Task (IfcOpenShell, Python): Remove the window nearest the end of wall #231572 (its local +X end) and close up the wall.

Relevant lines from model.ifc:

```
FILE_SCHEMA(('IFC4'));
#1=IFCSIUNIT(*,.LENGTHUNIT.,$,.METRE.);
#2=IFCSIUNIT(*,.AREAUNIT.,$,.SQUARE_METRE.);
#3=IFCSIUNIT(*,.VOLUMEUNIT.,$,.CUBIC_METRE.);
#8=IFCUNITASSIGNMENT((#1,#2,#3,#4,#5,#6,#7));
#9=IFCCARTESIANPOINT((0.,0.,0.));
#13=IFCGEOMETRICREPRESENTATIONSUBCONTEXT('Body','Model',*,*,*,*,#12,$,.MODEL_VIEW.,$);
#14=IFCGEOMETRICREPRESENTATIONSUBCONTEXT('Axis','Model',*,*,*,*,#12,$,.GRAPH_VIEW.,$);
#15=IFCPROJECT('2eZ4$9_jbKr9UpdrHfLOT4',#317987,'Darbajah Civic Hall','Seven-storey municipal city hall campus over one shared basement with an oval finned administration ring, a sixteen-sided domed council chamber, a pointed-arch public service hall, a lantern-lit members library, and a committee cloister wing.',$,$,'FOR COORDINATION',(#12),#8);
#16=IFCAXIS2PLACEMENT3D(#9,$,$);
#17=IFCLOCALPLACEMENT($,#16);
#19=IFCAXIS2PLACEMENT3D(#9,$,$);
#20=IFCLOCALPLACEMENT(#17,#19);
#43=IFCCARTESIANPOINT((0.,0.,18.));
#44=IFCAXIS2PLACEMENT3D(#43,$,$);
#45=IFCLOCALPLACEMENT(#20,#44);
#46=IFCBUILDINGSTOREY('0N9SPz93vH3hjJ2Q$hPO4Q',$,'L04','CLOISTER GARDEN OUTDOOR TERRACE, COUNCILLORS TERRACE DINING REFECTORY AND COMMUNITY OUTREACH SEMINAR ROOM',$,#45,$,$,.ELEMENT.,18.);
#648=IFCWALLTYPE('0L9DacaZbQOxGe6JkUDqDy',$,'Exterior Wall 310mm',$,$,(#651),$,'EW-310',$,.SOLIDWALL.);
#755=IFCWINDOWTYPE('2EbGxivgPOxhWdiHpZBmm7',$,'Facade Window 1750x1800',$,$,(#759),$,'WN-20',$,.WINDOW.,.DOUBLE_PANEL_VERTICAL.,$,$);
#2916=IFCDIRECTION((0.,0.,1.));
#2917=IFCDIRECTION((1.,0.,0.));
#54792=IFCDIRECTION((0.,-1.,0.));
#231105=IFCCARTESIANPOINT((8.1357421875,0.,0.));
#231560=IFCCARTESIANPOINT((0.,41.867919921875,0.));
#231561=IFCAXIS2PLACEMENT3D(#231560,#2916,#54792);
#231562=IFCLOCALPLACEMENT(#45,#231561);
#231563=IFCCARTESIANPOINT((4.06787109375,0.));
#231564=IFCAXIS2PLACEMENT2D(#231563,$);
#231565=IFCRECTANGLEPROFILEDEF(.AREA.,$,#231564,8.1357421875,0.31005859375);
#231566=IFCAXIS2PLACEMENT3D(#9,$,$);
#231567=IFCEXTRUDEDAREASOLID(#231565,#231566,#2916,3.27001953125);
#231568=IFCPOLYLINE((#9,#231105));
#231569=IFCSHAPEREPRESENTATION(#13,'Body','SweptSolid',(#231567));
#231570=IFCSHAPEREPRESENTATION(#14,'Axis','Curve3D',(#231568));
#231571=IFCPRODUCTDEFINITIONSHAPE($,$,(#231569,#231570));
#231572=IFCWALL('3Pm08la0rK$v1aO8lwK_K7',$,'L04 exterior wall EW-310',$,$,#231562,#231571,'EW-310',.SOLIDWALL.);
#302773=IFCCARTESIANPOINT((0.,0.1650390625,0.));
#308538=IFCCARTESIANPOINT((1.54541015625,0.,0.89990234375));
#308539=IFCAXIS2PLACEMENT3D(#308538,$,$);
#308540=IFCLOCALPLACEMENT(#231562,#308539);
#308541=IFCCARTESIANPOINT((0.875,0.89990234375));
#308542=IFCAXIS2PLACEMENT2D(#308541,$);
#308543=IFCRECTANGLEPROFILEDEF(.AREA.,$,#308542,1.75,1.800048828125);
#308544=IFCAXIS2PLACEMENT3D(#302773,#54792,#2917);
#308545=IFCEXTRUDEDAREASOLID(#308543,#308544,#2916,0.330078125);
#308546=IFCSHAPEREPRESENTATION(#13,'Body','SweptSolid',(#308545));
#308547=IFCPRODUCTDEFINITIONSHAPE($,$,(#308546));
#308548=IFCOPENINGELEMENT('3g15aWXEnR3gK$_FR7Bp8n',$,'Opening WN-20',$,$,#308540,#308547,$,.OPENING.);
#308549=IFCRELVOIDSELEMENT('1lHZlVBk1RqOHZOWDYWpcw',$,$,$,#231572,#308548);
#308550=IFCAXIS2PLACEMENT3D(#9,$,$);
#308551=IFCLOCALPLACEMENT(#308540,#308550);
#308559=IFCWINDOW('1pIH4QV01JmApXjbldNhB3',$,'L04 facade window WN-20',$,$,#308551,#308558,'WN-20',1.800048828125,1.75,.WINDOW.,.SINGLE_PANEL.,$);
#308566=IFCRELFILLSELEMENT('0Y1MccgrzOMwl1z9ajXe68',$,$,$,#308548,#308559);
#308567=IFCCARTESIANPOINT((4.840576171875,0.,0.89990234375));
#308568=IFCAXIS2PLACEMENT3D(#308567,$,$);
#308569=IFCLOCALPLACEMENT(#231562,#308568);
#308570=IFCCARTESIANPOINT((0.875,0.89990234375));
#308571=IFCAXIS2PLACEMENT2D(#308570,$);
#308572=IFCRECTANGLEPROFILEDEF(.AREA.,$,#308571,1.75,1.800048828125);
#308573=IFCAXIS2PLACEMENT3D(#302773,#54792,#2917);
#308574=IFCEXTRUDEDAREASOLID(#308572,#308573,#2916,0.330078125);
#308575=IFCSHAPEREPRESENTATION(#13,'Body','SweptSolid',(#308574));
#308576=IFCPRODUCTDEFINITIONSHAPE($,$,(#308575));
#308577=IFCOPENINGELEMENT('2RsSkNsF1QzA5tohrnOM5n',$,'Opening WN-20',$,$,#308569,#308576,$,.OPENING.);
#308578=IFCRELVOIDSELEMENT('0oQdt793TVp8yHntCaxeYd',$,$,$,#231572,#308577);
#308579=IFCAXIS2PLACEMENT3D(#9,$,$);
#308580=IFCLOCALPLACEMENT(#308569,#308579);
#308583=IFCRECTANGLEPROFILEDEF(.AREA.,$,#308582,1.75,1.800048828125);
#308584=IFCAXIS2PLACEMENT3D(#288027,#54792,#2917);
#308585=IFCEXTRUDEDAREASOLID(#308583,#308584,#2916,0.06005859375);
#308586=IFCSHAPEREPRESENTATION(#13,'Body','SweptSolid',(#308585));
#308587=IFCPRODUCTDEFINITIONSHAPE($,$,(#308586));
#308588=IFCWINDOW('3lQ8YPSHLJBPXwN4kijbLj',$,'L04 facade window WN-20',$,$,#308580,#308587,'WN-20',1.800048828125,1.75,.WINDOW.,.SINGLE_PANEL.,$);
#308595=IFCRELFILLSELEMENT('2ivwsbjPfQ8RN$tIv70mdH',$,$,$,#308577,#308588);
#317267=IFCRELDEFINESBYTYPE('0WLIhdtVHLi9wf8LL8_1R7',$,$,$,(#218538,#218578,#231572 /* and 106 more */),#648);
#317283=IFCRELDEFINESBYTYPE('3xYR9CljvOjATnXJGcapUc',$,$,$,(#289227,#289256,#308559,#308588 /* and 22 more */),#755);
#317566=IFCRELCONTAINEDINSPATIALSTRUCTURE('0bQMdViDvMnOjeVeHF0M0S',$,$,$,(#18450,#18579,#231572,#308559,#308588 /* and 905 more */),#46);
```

```python
import ifcopenshell
import ifcopenshell.api.feature
import ifcopenshell.api.root
import ifcopenshell.geom
import ifcopenshell.util.shape

model = ifcopenshell.open("model.ifc")
settings = ifcopenshell.geom.settings()


def volume(element):
    """Net volume in cubic metres, openings subtracted."""
    shape = ifcopenshell.geom.create_shape(settings, element)
    return ifcopenshell.util.shape.get_volume(shape.geometry)


window = model.by_guid("3lQ8YPSHLJBPXwN4kijbLj")
opening = window.FillsVoids[0].RelatingOpeningElement
wall = opening.VoidsElements[0].RelatingBuildingElement
before = volume(wall)

ifcopenshell.api.root.remove_product(model, product=window)
ifcopenshell.api.feature.remove_feature(model, feature=opening)

after = volume(wall)

print(f"wall volume {before:.3f} -> {after:.3f} m3")

model.write("model_v2.ifc")
```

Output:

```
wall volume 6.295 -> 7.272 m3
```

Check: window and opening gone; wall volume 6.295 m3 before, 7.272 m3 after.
